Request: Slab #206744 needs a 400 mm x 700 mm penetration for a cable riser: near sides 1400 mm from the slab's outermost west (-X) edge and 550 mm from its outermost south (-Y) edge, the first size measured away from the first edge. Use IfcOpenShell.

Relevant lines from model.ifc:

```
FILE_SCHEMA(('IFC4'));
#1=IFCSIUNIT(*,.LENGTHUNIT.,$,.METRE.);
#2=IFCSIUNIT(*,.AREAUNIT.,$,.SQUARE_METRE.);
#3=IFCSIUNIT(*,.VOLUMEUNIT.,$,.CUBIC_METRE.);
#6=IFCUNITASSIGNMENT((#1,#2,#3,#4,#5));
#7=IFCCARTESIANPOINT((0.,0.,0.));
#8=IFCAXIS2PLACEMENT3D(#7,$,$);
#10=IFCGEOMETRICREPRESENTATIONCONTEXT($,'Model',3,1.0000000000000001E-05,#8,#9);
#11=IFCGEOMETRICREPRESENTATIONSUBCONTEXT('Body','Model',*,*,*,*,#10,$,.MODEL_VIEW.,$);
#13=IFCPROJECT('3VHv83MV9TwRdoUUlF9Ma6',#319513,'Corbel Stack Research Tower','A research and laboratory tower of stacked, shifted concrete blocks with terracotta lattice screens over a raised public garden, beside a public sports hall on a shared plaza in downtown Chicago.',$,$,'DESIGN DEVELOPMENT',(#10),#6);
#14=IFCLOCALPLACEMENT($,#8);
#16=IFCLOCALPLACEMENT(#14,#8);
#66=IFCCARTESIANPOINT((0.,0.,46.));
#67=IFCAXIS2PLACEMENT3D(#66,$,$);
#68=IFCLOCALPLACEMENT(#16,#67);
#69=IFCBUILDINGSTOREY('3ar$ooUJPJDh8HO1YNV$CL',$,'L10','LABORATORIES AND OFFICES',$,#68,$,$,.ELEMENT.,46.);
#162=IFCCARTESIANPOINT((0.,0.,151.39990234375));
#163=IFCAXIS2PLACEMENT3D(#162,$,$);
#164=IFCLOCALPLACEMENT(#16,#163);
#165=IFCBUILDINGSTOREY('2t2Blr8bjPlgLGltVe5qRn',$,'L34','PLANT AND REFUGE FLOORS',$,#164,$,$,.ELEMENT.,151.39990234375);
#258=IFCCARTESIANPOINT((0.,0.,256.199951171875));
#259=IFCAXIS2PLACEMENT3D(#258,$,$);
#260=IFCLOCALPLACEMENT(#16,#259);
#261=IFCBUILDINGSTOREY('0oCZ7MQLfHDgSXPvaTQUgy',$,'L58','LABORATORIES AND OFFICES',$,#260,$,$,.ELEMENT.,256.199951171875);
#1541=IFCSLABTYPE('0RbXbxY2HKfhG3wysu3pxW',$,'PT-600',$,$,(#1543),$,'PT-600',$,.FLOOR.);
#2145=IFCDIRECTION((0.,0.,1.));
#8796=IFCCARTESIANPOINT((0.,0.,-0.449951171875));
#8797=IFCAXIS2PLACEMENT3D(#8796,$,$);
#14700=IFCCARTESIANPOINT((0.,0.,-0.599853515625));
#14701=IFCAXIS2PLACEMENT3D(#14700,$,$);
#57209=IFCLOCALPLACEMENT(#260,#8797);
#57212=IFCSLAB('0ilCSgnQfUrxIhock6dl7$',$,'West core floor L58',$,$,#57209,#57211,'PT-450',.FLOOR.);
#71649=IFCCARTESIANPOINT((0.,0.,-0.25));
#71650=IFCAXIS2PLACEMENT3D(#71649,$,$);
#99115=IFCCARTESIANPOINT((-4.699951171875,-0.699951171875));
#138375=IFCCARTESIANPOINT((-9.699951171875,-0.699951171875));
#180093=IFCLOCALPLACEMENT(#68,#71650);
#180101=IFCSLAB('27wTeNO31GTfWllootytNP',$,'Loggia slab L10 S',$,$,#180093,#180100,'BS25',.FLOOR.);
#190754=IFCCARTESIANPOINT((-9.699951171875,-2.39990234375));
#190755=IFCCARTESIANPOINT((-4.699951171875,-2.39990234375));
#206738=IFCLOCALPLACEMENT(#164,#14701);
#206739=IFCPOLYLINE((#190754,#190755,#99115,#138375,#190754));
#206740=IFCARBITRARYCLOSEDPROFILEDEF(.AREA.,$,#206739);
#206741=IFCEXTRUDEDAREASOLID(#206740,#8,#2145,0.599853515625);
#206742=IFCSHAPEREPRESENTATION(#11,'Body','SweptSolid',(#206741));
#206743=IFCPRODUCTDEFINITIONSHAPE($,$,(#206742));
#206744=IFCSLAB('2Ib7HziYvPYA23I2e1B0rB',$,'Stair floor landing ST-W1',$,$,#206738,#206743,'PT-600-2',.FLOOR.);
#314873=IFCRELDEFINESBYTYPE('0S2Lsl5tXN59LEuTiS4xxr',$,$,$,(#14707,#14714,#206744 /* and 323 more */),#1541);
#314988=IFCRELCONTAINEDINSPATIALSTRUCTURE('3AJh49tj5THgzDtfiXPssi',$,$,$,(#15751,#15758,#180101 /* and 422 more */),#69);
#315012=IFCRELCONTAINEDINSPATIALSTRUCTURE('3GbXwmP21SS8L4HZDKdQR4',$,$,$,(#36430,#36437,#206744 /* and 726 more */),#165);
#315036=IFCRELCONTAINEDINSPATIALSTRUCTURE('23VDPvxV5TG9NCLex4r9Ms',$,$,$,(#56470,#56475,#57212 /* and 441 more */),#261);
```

```python
import numpy as np
import ifcopenshell
import ifcopenshell.api.feature
import ifcopenshell.api.geometry
import ifcopenshell.api.root
import ifcopenshell.geom
import ifcopenshell.util.placement
import ifcopenshell.util.representation
import ifcopenshell.util.shape
import ifcopenshell.util.unit

model = ifcopenshell.open("model.ifc")
unit_scale = ifcopenshell.util.unit.calculate_unit_scale(model)
settings = ifcopenshell.geom.settings()


def volume(element):
    """Net volume in cubic metres, openings subtracted."""
    shape = ifcopenshell.geom.create_shape(settings, element)
    return ifcopenshell.util.shape.get_volume(shape.geometry)


slab = model.by_guid("2Ib7HziYvPYA23I2e1B0rB")
before = volume(slab)

# Extent in the slab's own axes, in metres. The edges named are its -X and -Y sides.
slab_shape = ifcopenshell.geom.create_shape(settings, slab)
vertices = ifcopenshell.util.shape.get_vertices(slab_shape.geometry)
x_min, y_min, bottom = vertices.min(axis=0)
top = vertices[:, 2].max()

opening = ifcopenshell.api.root.create_entity(model, ifc_class="IfcOpeningElement", name="Cable riser opening", predefined_type="OPENING")
context = ifcopenshell.util.representation.get_context(model, "Model", "Body", "MODEL_VIEW")
width, depth = 0.4, 0.7
outline = [(0.0, 0.0), (width, 0.0), (width, depth), (0.0, depth), (0.0, 0.0)]
# Overshoot both faces by 50 mm so the cut is clean.
shape = ifcopenshell.api.geometry.add_slab_representation(
    model, context=context, depth=top - bottom + 0.1, polyline=outline
)
ifcopenshell.api.geometry.assign_representation(model, product=opening, representation=shape)

matrix = ifcopenshell.util.placement.get_local_placement(slab.ObjectPlacement)
matrix[:, 3] = matrix @ np.append(np.array([x_min + 1.4, y_min + 0.55, bottom - 0.05]) / unit_scale, 1.0)
ifcopenshell.api.geometry.edit_object_placement(model, product=opening, matrix=matrix, is_si=False)
ifcopenshell.api.feature.add_feature(model, feature=opening, element=slab)

after = volume(slab)

print(f"slab volume {before:.3f} -> {after:.3f} m3")

model.write("model_rev.ifc")
```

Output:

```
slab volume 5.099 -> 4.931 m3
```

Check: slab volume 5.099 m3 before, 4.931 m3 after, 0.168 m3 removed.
